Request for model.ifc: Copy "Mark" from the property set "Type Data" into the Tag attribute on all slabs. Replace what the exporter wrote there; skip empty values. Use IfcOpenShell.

First a look at what the model holds.

```python
import ifcopenshell
import ifcopenshell.util.element

model = ifcopenshell.open("model.ifc")
print(model.schema)
slabs = model.by_type("IfcSlab")
print(len(slabs), "slabs")
for e in slabs[:8]:
    source = ifcopenshell.util.element.get_pset(e, "Type Data", "Mark")
    target = e.Tag
    print(e.id(), repr(source), repr(target), sep=" | ")
```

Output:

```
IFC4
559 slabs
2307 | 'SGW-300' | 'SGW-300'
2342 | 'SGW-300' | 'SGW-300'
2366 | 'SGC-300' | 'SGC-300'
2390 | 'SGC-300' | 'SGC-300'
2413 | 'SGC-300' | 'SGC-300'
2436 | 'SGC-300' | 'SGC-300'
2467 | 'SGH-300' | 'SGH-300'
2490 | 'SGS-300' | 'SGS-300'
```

```python
import ifcopenshell
import ifcopenshell.util.element

model = ifcopenshell.open("model.ifc")

count = 0
for e in model.by_type("IfcSlab"):
    value = ifcopenshell.util.element.get_pset(e, "Type Data", "Mark")
    current = e.Tag
    if not value or not value.strip() or current == value:
        continue
    e.Tag = value
    count += 1

print(count, "slabs updated")

model.write("model_updated.ifc")
```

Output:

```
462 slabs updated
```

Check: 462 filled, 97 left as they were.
